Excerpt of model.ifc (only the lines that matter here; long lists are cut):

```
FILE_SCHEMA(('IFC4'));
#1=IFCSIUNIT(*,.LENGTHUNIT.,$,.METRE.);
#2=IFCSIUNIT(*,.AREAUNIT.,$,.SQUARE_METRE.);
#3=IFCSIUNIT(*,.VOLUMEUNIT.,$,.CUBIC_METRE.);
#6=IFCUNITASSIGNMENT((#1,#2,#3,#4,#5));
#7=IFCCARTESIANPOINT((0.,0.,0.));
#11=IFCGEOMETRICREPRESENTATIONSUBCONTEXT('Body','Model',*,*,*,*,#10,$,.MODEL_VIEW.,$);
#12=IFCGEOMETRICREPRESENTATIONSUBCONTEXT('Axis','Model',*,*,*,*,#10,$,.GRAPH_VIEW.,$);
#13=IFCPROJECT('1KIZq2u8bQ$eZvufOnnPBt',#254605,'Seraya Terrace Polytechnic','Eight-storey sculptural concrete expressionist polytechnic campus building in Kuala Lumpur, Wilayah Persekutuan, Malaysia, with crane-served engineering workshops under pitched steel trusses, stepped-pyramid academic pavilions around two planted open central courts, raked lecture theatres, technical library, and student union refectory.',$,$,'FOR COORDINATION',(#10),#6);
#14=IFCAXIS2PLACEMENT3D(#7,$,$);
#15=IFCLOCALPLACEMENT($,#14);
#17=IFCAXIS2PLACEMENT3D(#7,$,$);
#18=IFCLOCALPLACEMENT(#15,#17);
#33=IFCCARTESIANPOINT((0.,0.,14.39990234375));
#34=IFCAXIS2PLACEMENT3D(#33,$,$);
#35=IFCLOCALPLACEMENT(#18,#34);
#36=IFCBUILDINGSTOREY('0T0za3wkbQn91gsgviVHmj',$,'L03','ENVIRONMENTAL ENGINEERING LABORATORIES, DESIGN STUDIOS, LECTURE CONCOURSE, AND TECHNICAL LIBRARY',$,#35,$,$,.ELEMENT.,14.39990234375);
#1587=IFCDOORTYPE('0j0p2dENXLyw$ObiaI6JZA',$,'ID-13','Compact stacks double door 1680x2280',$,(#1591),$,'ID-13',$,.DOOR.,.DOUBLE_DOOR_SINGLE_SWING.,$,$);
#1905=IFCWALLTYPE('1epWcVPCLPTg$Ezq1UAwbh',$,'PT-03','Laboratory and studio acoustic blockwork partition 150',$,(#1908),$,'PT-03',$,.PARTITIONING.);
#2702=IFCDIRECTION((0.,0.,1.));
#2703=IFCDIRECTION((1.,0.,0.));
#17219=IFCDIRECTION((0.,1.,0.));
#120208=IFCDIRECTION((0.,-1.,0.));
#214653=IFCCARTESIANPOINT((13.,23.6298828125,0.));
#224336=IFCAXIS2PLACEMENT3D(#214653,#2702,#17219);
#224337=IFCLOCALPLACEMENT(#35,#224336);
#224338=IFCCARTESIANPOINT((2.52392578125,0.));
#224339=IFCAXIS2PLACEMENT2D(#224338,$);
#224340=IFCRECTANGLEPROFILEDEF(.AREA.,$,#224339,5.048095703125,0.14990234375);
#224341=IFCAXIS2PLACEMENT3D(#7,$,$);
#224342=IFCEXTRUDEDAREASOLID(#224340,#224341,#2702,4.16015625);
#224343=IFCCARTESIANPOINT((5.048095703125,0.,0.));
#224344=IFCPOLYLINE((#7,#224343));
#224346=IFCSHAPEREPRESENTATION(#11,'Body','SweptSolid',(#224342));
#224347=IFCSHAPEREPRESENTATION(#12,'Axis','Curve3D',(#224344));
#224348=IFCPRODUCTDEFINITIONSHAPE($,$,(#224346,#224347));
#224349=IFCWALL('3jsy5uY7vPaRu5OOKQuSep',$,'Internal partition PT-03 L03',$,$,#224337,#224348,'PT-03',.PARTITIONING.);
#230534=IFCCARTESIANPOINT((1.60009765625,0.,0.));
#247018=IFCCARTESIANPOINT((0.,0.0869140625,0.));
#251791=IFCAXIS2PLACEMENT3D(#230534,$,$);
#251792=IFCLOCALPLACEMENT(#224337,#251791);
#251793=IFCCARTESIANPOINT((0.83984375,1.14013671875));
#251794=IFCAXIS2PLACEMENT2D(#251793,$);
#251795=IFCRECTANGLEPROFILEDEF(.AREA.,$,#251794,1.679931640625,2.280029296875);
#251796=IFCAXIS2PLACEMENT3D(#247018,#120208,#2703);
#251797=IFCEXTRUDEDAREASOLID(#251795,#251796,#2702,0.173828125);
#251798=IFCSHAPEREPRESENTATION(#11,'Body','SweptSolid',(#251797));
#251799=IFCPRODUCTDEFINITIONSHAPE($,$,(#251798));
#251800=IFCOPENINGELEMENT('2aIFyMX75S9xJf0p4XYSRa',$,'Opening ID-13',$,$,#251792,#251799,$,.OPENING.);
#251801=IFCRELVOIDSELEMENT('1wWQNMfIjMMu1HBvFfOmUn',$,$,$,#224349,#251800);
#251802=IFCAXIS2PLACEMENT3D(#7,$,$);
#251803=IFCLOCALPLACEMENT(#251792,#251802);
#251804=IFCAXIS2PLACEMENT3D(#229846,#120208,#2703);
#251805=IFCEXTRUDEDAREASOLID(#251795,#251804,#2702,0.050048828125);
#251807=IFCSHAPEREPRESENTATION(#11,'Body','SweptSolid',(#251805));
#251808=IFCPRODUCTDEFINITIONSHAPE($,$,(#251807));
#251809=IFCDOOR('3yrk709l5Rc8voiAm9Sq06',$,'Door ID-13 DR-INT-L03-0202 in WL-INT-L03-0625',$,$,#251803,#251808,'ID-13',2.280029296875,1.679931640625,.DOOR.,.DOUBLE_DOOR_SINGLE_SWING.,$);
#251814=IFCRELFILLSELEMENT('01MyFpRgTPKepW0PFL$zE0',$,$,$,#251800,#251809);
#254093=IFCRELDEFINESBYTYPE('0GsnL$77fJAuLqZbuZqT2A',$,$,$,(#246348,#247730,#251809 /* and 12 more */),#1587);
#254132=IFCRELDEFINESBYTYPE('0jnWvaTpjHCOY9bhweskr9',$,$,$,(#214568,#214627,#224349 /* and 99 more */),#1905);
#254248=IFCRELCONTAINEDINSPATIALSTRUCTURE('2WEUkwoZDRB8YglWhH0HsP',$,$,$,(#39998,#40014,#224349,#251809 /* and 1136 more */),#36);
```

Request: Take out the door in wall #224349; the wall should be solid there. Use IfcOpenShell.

```python
import ifcopenshell
import ifcopenshell.api.feature
import ifcopenshell.api.root
import ifcopenshell.geom
import ifcopenshell.util.shape

model = ifcopenshell.open("model.ifc")
settings = ifcopenshell.geom.settings()


def volume(element):
    """Net volume in cubic metres, openings subtracted."""
    shape = ifcopenshell.geom.create_shape(settings, element)
    return ifcopenshell.util.shape.get_volume(shape.geometry)


door = model.by_guid("3yrk709l5Rc8voiAm9Sq06")
opening = door.FillsVoids[0].RelatingOpeningElement
wall = opening.VoidsElements[0].RelatingBuildingElement
before = volume(wall)

ifcopenshell.api.root.remove_product(model, product=door)
ifcopenshell.api.feature.remove_feature(model, feature=opening)

after = volume(wall)

print(f"wall volume {before:.3f} -> {after:.3f} m3")

model.write("model_updated.ifc")
```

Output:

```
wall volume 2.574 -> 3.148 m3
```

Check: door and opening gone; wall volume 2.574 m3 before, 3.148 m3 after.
